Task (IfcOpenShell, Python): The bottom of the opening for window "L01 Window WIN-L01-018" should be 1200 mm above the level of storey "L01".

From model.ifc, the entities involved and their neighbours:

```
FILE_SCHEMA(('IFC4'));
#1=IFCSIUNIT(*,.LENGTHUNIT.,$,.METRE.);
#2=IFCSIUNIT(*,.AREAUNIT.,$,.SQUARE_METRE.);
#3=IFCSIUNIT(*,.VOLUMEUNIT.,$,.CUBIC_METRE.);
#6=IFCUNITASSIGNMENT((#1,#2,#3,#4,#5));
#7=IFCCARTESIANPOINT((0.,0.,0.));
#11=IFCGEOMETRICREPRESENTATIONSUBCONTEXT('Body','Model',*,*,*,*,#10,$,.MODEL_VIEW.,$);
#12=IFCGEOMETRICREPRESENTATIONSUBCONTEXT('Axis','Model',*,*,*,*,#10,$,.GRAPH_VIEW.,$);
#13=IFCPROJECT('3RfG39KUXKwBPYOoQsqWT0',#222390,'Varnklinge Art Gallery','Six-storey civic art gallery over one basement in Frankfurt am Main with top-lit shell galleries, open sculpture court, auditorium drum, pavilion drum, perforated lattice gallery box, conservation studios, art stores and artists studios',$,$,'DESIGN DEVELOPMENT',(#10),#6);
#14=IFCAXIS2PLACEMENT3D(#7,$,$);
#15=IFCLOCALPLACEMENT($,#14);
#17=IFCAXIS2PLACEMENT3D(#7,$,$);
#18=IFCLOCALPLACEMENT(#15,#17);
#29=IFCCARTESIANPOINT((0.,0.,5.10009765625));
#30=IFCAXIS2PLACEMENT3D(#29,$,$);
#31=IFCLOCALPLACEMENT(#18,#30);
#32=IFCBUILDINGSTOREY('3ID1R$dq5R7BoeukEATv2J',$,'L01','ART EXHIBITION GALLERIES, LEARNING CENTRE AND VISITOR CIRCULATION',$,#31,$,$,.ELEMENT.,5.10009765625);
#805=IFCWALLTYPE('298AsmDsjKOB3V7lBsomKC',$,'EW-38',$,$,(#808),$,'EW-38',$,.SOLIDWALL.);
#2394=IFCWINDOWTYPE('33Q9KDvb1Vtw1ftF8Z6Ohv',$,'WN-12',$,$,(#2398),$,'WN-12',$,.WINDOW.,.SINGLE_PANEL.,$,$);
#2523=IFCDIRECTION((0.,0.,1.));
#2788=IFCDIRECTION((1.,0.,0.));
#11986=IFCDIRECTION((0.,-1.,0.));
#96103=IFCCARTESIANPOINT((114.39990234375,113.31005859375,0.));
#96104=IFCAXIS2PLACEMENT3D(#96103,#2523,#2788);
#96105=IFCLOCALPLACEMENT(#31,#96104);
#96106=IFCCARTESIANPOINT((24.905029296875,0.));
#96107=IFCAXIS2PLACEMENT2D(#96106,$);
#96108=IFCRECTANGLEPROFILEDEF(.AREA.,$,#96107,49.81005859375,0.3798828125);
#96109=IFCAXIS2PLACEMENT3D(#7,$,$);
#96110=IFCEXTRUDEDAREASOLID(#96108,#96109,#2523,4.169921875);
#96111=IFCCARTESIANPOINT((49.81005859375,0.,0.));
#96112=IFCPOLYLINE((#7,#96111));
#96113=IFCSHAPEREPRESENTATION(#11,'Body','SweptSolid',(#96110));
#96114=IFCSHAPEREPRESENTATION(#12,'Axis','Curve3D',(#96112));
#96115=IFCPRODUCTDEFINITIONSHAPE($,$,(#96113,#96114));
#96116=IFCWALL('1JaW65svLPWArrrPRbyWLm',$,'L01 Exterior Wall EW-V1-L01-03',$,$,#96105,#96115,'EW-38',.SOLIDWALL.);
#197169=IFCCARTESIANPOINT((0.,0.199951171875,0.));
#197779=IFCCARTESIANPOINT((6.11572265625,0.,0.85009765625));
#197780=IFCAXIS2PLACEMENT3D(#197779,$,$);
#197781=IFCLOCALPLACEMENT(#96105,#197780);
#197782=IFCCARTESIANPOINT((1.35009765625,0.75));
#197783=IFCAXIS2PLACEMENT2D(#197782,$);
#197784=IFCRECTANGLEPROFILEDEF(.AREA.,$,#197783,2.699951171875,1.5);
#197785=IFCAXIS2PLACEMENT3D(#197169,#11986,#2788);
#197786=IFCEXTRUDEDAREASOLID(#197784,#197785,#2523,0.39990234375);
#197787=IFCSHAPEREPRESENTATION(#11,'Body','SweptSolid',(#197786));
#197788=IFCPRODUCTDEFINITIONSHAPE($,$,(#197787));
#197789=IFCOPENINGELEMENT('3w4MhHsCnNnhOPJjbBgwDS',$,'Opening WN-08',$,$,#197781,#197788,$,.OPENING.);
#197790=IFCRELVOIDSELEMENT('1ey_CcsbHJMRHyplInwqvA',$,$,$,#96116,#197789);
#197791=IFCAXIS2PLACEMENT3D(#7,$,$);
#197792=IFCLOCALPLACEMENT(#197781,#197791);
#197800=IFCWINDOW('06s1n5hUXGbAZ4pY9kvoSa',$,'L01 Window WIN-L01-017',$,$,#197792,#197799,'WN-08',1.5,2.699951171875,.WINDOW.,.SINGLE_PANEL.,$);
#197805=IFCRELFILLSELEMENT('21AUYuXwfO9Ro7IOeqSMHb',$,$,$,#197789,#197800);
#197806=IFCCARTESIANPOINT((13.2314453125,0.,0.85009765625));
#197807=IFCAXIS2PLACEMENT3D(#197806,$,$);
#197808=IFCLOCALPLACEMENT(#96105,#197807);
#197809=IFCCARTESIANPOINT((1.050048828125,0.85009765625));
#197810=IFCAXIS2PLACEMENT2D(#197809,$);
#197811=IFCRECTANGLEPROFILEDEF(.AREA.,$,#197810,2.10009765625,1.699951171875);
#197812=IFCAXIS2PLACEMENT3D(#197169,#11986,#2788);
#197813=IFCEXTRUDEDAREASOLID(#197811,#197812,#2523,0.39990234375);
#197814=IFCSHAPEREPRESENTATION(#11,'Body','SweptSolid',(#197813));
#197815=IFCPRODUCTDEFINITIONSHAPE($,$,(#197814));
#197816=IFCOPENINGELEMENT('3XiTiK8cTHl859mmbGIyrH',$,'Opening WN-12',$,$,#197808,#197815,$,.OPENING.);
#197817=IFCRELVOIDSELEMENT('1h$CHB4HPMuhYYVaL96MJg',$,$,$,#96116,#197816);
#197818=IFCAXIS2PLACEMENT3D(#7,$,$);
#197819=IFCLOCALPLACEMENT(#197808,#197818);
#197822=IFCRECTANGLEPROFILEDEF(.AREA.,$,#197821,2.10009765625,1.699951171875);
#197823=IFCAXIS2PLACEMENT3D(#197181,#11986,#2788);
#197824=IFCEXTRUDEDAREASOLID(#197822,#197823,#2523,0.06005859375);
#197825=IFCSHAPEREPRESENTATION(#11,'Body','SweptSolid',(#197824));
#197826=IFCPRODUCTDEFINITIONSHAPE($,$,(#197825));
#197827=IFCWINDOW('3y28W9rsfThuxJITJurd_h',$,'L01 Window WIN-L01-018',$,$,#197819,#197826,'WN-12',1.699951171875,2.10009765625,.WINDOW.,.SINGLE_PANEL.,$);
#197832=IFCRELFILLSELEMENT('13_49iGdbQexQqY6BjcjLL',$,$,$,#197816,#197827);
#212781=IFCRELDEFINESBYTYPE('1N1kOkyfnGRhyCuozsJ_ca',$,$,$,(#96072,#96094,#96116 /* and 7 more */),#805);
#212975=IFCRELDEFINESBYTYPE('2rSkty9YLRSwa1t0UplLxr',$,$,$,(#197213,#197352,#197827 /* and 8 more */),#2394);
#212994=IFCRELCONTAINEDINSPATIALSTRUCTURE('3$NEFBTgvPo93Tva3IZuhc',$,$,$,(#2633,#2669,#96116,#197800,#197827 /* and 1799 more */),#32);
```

```python
import numpy as np
import ifcopenshell
import ifcopenshell.api.geometry
import ifcopenshell.geom
import ifcopenshell.util.element
import ifcopenshell.util.placement
import ifcopenshell.util.shape
import ifcopenshell.util.unit

model = ifcopenshell.open("model.ifc")
unit_scale = ifcopenshell.util.unit.calculate_unit_scale(model)

window = model.by_id(197827)
opening = window.FillsVoids[0].RelatingOpeningElement
storey = ifcopenshell.util.element.get_container(window, ifc_class="IfcBuildingStorey")
level = ifcopenshell.util.placement.get_local_placement(storey.ObjectPlacement)[2, 3]

# The opening's origin need not be at the sill, so measure its lowest point.
shape = ifcopenshell.geom.create_shape(ifcopenshell.geom.settings(), opening)
bottom = ifcopenshell.util.shape.get_shape_bottom_elevation(shape, shape.geometry) / unit_scale
dz = level + 1.2 - bottom

shift = np.array([0.0, 0.0, dz])
# The window is placed relative to its opening, so it follows when the opening moves.
matrix = ifcopenshell.util.placement.get_local_placement(opening.ObjectPlacement)
matrix[:3, 3] += shift
ifcopenshell.api.geometry.edit_object_placement(
    model, product=opening, matrix=matrix, is_si=False, should_transform_children=True
)

print(f"moved by {dz * unit_scale:+.3f} m")

model.write("model_v2.ifc")
```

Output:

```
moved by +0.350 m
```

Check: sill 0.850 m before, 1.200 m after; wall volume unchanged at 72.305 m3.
